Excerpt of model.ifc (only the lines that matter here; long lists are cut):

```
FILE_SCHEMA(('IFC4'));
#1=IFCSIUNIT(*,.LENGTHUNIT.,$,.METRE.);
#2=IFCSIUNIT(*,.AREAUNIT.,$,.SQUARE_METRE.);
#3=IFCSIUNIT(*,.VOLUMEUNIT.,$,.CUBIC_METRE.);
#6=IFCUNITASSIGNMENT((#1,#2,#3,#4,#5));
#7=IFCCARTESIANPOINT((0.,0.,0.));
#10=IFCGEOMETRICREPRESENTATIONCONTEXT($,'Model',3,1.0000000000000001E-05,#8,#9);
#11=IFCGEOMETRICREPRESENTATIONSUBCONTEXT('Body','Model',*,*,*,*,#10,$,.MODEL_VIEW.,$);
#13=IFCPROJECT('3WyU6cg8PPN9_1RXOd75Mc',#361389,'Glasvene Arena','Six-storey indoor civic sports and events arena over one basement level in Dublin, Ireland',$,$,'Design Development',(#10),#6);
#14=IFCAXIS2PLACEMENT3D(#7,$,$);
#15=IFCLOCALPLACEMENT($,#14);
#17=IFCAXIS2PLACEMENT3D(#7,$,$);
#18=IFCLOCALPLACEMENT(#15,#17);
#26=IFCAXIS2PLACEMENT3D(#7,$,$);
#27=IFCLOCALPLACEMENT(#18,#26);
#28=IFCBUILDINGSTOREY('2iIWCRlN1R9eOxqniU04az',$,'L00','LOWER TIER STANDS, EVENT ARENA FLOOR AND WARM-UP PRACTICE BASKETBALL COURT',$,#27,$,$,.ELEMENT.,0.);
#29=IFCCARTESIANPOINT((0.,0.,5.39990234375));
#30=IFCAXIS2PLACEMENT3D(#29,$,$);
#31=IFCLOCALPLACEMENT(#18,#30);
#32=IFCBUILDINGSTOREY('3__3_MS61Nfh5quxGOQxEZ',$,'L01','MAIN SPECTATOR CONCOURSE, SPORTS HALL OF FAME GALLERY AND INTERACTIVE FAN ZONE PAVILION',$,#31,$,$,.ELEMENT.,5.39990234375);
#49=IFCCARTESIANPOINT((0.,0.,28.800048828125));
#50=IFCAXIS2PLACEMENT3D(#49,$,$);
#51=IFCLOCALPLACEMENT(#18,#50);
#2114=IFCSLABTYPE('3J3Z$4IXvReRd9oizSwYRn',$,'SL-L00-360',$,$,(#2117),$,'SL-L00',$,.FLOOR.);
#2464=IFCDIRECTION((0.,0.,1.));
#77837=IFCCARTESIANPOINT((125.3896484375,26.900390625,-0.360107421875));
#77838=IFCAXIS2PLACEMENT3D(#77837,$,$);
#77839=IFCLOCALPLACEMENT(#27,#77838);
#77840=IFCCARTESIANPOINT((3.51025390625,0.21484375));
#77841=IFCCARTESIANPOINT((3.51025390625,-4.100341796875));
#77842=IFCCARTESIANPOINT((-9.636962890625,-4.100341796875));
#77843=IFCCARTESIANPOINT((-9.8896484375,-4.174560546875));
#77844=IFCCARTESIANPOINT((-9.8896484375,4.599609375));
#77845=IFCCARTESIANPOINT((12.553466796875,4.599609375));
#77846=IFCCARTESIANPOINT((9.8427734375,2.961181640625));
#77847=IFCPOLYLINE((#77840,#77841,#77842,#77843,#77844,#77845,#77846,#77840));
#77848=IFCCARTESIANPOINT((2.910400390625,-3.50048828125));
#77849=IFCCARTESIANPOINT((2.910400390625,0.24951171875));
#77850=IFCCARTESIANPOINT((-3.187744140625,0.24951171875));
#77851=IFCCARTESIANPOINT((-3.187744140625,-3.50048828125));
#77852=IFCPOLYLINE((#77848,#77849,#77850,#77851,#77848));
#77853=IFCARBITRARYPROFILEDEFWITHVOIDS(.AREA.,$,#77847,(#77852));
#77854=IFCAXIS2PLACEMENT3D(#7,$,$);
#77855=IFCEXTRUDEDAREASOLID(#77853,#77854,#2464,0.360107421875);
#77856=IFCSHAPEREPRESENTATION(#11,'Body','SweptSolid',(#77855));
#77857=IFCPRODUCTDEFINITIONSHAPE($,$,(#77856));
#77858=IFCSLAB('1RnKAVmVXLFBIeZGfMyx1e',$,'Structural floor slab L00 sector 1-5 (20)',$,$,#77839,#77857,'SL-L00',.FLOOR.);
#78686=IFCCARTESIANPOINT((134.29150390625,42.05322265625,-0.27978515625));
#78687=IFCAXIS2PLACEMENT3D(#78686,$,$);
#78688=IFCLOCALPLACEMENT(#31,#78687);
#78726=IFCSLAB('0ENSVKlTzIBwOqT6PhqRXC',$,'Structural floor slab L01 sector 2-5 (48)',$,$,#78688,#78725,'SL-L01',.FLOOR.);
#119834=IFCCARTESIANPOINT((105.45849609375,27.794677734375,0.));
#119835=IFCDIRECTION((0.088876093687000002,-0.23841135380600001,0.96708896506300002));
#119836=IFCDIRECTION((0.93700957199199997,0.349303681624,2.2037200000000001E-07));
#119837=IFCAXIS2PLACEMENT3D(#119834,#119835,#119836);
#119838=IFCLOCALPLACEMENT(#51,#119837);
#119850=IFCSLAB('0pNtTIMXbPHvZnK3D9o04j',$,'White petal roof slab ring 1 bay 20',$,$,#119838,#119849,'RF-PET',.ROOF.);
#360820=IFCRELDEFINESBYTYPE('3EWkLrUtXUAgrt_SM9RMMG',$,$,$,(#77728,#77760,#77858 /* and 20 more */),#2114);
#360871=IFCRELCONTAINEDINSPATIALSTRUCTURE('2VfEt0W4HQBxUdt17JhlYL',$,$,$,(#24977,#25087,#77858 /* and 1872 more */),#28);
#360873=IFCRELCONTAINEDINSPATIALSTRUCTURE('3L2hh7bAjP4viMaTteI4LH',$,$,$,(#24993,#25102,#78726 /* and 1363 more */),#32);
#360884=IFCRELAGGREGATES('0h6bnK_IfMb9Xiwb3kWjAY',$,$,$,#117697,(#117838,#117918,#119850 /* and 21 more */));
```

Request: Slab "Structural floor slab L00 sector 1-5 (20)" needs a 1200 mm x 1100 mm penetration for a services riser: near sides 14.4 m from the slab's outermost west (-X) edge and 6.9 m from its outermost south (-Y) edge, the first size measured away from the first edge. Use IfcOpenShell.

```python
import numpy as np
import ifcopenshell
import ifcopenshell.api.feature
import ifcopenshell.api.geometry
import ifcopenshell.api.root
import ifcopenshell.geom
import ifcopenshell.util.placement
import ifcopenshell.util.representation
import ifcopenshell.util.shape
import ifcopenshell.util.unit

model = ifcopenshell.open("model.ifc")
unit_scale = ifcopenshell.util.unit.calculate_unit_scale(model)
settings = ifcopenshell.geom.settings()


def volume(element):
    """Net volume in cubic metres, openings subtracted."""
    shape = ifcopenshell.geom.create_shape(settings, element)
    return ifcopenshell.util.shape.get_volume(shape.geometry)


slab = model.by_guid("1RnKAVmVXLFBIeZGfMyx1e")
before = volume(slab)

# Extent in the slab's own axes, in metres. The edges named are its -X and -Y sides.
slab_shape = ifcopenshell.geom.create_shape(settings, slab)
vertices = ifcopenshell.util.shape.get_vertices(slab_shape.geometry)
x_min, y_min, bottom = vertices.min(axis=0)
top = vertices[:, 2].max()

opening = ifcopenshell.api.root.create_entity(model, ifc_class="IfcOpeningElement", name="Services riser opening", predefined_type="OPENING")
context = ifcopenshell.util.representation.get_context(model, "Model", "Body", "MODEL_VIEW")
width, depth = 1.2, 1.1
outline = [(0.0, 0.0), (width, 0.0), (width, depth), (0.0, depth), (0.0, 0.0)]
# Overshoot both faces by 50 mm so the cut is clean.
shape = ifcopenshell.api.geometry.add_slab_representation(
    model, context=context, depth=top - bottom + 0.1, polyline=outline
)
ifcopenshell.api.geometry.assign_representation(model, product=opening, representation=shape)

matrix = ifcopenshell.util.placement.get_local_placement(slab.ObjectPlacement)
matrix[:, 3] = matrix @ np.append(np.array([x_min + 14.4, y_min + 6.9, bottom - 0.05]) / unit_scale, 1.0)
ifcopenshell.api.geometry.edit_object_placement(model, product=opening, matrix=matrix, is_si=False)
ifcopenshell.api.feature.add_feature(model, feature=opening, element=slab)

after = volume(slab)

print(f"slab volume {before:.3f} -> {after:.3f} m3")

model.write("model_edited.ifc")
```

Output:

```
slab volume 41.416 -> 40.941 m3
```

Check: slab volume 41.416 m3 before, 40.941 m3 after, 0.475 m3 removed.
